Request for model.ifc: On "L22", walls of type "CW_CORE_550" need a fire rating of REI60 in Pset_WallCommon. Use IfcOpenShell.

First a look at what the model holds.

```python
import ifcopenshell
import ifcopenshell.util.element

model = ifcopenshell.open("model.ifc")
print(model.schema)
storey = next(s for s in model.by_type("IfcBuildingStorey") if s.Name == "L22")
walls = [e for e in ifcopenshell.util.element.get_decomposition(storey) if e.is_a("IfcWall")]
seen = {}
for e in walls:
    element_type = ifcopenshell.util.element.get_type(e)
    key = (element_type.Name if element_type != e and element_type else None, ifcopenshell.util.element.get_pset(e, "Pset_WallCommon", "FireRating"))
    seen[key] = seen.get(key, 0) + 1
for (name, value), count in sorted(seen.items(), key=str):
    print(count, "x", name, "|", value)
```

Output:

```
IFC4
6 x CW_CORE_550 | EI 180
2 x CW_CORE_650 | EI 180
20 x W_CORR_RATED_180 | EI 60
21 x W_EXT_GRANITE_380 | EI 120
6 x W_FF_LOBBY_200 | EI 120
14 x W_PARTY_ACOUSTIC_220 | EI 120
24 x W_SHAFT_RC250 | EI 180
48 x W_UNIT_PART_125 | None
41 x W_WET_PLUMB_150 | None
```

```python
import ifcopenshell
import ifcopenshell.api.pset
import ifcopenshell.util.element

model = ifcopenshell.open("model.ifc")

storey = next(s for s in model.by_type("IfcBuildingStorey") if s.Name == "L22")
walls = [e for e in ifcopenshell.util.element.get_decomposition(storey) if e.is_a("IfcWall")]

count = 0
for e in walls:
    element_type = ifcopenshell.util.element.get_type(e)
    if element_type in (None, e) or element_type.Name != "CW_CORE_550":
        continue
    found = ifcopenshell.util.element.get_pset(e, "Pset_WallCommon", should_inherit=False)
    if found:
        pset = model.by_id(found["id"])
        if len(ifcopenshell.util.element.get_elements_by_pset(pset)) > 1:
            pset = ifcopenshell.api.pset.unshare_pset(model, products=[e], pset=pset)[0]
    else:
        pset = ifcopenshell.api.pset.add_pset(model, product=e, name="Pset_WallCommon")
    ifcopenshell.api.pset.edit_pset(model, pset=pset, properties={"FireRating": "REI60"})
    count += 1

print(count, "walls updated")

model.write("model_v2.ifc")
```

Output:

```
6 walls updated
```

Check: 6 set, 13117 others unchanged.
